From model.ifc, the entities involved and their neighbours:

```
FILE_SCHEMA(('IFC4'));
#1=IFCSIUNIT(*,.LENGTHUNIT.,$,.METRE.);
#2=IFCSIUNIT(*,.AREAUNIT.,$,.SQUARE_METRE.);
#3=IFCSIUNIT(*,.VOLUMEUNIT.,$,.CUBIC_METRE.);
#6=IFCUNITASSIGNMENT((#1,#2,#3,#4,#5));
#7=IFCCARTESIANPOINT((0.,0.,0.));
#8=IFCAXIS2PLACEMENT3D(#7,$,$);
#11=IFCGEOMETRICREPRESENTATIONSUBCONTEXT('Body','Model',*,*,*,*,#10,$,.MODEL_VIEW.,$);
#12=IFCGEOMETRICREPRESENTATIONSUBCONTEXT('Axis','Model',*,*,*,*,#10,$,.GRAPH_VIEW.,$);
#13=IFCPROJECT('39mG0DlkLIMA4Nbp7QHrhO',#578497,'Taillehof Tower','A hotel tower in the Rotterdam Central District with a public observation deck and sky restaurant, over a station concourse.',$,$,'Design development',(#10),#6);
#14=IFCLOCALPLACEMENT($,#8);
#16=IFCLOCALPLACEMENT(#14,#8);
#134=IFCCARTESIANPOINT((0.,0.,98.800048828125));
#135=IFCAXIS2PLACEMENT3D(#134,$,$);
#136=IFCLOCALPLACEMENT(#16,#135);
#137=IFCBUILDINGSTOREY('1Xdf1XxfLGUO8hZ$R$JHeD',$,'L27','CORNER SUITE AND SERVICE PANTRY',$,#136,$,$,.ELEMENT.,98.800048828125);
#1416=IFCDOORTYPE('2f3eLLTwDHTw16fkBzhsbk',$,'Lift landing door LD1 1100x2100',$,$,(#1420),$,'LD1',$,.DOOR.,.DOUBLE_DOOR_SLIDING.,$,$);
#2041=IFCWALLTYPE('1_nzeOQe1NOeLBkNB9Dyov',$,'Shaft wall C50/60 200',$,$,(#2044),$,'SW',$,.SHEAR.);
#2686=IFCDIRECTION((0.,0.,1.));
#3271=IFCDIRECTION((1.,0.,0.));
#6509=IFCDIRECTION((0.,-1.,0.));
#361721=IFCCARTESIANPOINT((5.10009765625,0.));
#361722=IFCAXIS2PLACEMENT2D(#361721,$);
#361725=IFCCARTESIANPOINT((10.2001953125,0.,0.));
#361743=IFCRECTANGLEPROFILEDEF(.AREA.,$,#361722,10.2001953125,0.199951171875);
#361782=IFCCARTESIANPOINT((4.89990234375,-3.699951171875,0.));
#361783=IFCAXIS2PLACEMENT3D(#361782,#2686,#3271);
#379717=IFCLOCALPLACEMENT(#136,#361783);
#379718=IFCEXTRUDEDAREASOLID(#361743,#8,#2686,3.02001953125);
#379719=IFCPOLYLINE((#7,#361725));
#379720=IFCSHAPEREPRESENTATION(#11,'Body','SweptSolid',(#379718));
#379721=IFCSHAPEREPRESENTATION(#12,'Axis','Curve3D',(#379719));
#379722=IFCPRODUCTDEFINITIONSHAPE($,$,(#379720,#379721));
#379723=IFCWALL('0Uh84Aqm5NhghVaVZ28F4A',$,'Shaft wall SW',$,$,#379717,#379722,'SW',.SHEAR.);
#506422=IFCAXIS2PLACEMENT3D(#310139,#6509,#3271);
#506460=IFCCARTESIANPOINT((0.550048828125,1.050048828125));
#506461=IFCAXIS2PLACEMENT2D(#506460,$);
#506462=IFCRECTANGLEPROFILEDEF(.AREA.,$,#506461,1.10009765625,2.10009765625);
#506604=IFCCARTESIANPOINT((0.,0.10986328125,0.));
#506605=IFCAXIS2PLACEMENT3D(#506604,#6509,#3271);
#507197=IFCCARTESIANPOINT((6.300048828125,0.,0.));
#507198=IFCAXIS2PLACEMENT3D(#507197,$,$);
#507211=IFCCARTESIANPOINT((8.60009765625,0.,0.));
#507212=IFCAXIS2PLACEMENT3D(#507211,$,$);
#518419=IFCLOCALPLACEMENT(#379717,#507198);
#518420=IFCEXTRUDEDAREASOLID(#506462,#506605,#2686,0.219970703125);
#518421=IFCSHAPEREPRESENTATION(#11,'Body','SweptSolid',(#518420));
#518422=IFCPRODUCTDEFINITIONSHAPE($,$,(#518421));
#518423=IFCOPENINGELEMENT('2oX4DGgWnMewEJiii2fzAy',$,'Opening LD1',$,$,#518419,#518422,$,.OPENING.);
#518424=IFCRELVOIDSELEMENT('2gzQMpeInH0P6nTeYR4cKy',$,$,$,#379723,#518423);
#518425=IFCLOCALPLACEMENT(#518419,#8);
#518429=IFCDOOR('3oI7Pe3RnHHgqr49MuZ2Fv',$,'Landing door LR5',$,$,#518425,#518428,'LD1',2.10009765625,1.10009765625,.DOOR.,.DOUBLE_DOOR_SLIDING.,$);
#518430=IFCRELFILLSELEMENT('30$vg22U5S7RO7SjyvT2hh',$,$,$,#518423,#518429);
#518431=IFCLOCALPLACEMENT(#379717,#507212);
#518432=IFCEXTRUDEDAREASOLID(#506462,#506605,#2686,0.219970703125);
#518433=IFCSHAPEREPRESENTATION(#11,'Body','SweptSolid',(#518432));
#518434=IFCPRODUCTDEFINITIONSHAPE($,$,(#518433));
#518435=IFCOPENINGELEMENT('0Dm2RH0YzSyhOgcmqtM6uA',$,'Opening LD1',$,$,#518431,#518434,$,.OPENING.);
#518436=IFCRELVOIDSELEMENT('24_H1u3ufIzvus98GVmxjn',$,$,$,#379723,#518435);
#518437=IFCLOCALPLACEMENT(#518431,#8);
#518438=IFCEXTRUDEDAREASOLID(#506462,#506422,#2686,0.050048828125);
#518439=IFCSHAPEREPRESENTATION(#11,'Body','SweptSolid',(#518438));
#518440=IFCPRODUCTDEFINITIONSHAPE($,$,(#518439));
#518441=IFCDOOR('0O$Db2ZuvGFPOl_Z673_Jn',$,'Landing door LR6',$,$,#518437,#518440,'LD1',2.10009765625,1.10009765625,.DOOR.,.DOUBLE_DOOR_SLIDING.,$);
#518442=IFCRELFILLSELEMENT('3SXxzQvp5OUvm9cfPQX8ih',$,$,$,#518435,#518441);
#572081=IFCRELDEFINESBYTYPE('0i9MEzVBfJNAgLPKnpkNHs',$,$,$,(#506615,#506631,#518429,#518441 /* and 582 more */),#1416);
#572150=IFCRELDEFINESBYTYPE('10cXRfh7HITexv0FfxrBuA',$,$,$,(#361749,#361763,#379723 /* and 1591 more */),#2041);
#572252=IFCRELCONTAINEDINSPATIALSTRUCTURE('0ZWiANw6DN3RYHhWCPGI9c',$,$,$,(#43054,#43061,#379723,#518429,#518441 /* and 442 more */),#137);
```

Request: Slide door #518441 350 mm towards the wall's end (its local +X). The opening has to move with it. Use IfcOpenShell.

```python
import ifcopenshell
import ifcopenshell.api.geometry
import ifcopenshell.util.placement
import ifcopenshell.util.unit

model = ifcopenshell.open("model.ifc")
unit_scale = ifcopenshell.util.unit.calculate_unit_scale(model)

door = model.by_guid("0O$Db2ZuvGFPOl_Z673_Jn")
opening = door.FillsVoids[0].RelatingOpeningElement
wall = opening.VoidsElements[0].RelatingBuildingElement

wall_matrix = ifcopenshell.util.placement.get_local_placement(wall.ObjectPlacement)
shift = wall_matrix[:3, 0] * 0.35 / unit_scale
before = ifcopenshell.util.placement.get_local_placement(door.ObjectPlacement)[:3, 3].copy()

# The door is placed relative to its opening, so it follows when the opening moves.
matrix = ifcopenshell.util.placement.get_local_placement(opening.ObjectPlacement)
matrix[:3, 3] += shift
ifcopenshell.api.geometry.edit_object_placement(
    model, product=opening, matrix=matrix, is_si=False, should_transform_children=True
)

after = ifcopenshell.util.placement.get_local_placement(door.ObjectPlacement)[:3, 3]
print("door moved by", (after - before).round(3) + 0.0)

model.write("model_updated.ifc")
```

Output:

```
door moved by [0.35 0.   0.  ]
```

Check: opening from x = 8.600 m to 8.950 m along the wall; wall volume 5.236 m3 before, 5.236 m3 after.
